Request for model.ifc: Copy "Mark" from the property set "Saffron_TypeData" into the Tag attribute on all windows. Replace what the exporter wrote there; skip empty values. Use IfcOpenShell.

First a look at what the model holds.

```python
import ifcopenshell
import ifcopenshell.util.element

model = ifcopenshell.open("model.ifc")
print(model.schema)
windows = model.by_type("IfcWindow")
print(len(windows), "windows")
for e in windows[:8]:
    source = ifcopenshell.util.element.get_pset(e, "Saffron_TypeData", "Mark")
    target = e.Tag
    print(e.id(), repr(source), repr(target), sep=" | ")
```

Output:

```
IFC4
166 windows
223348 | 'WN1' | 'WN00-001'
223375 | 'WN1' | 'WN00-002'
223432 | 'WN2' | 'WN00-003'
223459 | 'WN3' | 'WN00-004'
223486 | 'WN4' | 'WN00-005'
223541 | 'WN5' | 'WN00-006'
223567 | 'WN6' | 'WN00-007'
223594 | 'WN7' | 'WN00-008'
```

```python
import ifcopenshell
import ifcopenshell.util.element

model = ifcopenshell.open("model.ifc")

count = 0
for e in model.by_type("IfcWindow"):
    value = ifcopenshell.util.element.get_pset(e, "Saffron_TypeData", "Mark")
    current = e.Tag
    if not value or not value.strip() or current == value:
        continue
    e.Tag = value
    count += 1

print(count, "windows updated")

model.write("model_updated.ifc")
```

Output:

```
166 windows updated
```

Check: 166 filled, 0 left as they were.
